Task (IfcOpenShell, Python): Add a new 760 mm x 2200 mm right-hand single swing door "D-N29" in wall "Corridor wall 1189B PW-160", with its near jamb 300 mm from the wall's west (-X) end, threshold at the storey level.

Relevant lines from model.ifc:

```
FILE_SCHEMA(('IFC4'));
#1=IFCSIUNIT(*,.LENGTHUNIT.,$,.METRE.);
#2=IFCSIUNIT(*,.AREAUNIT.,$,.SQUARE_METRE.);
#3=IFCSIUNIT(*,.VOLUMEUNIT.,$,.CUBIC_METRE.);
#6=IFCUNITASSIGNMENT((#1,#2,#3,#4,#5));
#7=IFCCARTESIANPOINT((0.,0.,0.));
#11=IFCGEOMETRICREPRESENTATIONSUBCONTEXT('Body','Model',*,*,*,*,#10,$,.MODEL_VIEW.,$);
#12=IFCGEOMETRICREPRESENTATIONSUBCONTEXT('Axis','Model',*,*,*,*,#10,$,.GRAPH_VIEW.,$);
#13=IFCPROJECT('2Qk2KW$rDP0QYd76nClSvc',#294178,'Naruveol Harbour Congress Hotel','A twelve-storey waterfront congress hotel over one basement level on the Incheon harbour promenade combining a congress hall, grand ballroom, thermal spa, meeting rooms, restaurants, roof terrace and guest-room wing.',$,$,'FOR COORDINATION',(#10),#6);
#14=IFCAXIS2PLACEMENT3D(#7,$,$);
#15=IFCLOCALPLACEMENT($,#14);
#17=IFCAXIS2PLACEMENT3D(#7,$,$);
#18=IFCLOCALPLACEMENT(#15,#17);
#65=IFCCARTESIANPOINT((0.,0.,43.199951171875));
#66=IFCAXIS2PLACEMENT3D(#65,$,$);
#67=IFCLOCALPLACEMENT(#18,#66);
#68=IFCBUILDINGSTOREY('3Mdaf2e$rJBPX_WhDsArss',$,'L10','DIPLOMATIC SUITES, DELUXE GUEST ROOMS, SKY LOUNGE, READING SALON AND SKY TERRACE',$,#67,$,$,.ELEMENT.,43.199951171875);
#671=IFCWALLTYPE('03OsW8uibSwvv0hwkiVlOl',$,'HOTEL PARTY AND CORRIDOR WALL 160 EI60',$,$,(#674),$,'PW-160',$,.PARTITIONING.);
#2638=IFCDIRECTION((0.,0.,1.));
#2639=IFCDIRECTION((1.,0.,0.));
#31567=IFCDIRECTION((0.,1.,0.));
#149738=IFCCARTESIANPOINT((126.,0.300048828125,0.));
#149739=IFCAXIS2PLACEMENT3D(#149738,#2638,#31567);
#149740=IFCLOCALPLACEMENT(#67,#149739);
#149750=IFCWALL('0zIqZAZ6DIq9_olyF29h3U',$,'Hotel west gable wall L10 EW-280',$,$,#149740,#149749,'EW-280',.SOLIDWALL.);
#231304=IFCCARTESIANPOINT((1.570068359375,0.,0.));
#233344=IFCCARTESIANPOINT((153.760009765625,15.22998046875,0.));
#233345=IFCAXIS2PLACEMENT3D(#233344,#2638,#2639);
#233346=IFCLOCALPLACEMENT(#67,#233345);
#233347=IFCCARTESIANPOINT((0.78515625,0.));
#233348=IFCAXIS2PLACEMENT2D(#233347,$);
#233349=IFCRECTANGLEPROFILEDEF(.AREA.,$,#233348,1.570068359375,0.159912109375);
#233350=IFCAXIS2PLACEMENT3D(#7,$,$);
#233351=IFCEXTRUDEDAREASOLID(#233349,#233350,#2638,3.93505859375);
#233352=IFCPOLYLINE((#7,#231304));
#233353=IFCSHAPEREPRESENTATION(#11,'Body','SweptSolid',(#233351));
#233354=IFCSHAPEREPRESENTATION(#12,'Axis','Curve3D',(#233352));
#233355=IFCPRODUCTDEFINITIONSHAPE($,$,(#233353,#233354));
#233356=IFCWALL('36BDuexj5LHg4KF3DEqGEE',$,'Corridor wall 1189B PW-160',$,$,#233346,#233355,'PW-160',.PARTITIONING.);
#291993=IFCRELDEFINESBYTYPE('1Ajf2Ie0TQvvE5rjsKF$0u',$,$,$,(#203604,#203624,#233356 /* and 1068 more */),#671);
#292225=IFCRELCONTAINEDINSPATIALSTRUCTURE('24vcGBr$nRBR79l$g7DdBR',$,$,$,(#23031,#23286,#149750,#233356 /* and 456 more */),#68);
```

```python
import numpy as np
import ifcopenshell
import ifcopenshell.api.feature
import ifcopenshell.api.geometry
import ifcopenshell.api.root
import ifcopenshell.api.spatial
import ifcopenshell.geom
import ifcopenshell.util.element
import ifcopenshell.util.placement
import ifcopenshell.util.representation
import ifcopenshell.util.shape
import ifcopenshell.util.unit

model = ifcopenshell.open("model.ifc")
unit_scale = ifcopenshell.util.unit.calculate_unit_scale(model)
settings = ifcopenshell.geom.settings()


def volume(element):
    """Net volume in cubic metres, openings subtracted."""
    shape = ifcopenshell.geom.create_shape(settings, element)
    return ifcopenshell.util.shape.get_volume(shape.geometry)


wall = model.by_guid("36BDuexj5LHg4KF3DEqGEE")
storey = ifcopenshell.util.element.get_container(wall, ifc_class="IfcBuildingStorey")
context = ifcopenshell.util.representation.get_context(model, "Model", "Body", "MODEL_VIEW")
before = volume(wall)

width, height, from_end, sill = 0.76, 2.2, 0.3, 0.0  # metres

# The wall runs along its own X axis, and the end named is its -X end.
wall_shape = ifcopenshell.geom.create_shape(settings, wall)
x, y, z = ifcopenshell.util.shape.get_vertices(wall_shape.geometry).T
start = x.min() + from_end
face, thickness = float(y.min()), float(y.max() - y.min())
wall_matrix = ifcopenshell.util.placement.get_local_placement(wall.ObjectPlacement)
level = ifcopenshell.util.placement.get_local_placement(storey.ObjectPlacement)[2, 3]


def in_wall(x, y):
    """Placement at x, y metres in the wall's axes, at sill height."""
    matrix = wall_matrix.copy()
    matrix[:, 3] = wall_matrix @ np.array([x / unit_scale, y / unit_scale, 0.0, 1.0])
    matrix[2, 3] = level + sill / unit_scale
    return matrix


# Opening: a box that overshoots both wall faces by 50 mm.
opening = ifcopenshell.api.root.create_entity(model, ifc_class="IfcOpeningElement", predefined_type="OPENING")
box = ifcopenshell.api.geometry.add_wall_representation(
    model, context=context, length=width, height=height, thickness=thickness + 0.1
)
ifcopenshell.api.geometry.assign_representation(model, product=opening, representation=box)
ifcopenshell.api.geometry.edit_object_placement(model, product=opening, matrix=in_wall(start, face - 0.05), is_si=False)
ifcopenshell.api.feature.add_feature(model, feature=opening, element=wall)

door = ifcopenshell.api.root.create_entity(model, ifc_class="IfcDoor", name="D-N29", predefined_type="DOOR")
door.OverallWidth, door.OverallHeight = width / unit_scale, height / unit_scale
door.OperationType = "SINGLE_SWING_RIGHT"
body = ifcopenshell.api.geometry.add_door_representation(
    model,
    context=context,
    overall_width=door.OverallWidth,
    overall_height=door.OverallHeight,
    operation_type="SINGLE_SWING_RIGHT",
    lining_properties={"LiningDepth": thickness / unit_scale, "ThresholdDepth": thickness / unit_scale},
)
ifcopenshell.api.geometry.assign_representation(model, product=door, representation=body)
ifcopenshell.api.spatial.assign_container(model, products=[door], relating_structure=storey)
ifcopenshell.api.feature.add_filling(model, opening=opening, element=door)

# The lining spans the wall, so the door starts at the wall face.
ifcopenshell.api.geometry.edit_object_placement(model, product=door, matrix=in_wall(start, face), is_si=False)

after = volume(wall)

print(f"wall volume {before:.3f} -> {after:.3f} m3")

model.write("model_edited.ifc")
```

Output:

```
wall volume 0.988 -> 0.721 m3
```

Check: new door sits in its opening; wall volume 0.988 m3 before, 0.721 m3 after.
